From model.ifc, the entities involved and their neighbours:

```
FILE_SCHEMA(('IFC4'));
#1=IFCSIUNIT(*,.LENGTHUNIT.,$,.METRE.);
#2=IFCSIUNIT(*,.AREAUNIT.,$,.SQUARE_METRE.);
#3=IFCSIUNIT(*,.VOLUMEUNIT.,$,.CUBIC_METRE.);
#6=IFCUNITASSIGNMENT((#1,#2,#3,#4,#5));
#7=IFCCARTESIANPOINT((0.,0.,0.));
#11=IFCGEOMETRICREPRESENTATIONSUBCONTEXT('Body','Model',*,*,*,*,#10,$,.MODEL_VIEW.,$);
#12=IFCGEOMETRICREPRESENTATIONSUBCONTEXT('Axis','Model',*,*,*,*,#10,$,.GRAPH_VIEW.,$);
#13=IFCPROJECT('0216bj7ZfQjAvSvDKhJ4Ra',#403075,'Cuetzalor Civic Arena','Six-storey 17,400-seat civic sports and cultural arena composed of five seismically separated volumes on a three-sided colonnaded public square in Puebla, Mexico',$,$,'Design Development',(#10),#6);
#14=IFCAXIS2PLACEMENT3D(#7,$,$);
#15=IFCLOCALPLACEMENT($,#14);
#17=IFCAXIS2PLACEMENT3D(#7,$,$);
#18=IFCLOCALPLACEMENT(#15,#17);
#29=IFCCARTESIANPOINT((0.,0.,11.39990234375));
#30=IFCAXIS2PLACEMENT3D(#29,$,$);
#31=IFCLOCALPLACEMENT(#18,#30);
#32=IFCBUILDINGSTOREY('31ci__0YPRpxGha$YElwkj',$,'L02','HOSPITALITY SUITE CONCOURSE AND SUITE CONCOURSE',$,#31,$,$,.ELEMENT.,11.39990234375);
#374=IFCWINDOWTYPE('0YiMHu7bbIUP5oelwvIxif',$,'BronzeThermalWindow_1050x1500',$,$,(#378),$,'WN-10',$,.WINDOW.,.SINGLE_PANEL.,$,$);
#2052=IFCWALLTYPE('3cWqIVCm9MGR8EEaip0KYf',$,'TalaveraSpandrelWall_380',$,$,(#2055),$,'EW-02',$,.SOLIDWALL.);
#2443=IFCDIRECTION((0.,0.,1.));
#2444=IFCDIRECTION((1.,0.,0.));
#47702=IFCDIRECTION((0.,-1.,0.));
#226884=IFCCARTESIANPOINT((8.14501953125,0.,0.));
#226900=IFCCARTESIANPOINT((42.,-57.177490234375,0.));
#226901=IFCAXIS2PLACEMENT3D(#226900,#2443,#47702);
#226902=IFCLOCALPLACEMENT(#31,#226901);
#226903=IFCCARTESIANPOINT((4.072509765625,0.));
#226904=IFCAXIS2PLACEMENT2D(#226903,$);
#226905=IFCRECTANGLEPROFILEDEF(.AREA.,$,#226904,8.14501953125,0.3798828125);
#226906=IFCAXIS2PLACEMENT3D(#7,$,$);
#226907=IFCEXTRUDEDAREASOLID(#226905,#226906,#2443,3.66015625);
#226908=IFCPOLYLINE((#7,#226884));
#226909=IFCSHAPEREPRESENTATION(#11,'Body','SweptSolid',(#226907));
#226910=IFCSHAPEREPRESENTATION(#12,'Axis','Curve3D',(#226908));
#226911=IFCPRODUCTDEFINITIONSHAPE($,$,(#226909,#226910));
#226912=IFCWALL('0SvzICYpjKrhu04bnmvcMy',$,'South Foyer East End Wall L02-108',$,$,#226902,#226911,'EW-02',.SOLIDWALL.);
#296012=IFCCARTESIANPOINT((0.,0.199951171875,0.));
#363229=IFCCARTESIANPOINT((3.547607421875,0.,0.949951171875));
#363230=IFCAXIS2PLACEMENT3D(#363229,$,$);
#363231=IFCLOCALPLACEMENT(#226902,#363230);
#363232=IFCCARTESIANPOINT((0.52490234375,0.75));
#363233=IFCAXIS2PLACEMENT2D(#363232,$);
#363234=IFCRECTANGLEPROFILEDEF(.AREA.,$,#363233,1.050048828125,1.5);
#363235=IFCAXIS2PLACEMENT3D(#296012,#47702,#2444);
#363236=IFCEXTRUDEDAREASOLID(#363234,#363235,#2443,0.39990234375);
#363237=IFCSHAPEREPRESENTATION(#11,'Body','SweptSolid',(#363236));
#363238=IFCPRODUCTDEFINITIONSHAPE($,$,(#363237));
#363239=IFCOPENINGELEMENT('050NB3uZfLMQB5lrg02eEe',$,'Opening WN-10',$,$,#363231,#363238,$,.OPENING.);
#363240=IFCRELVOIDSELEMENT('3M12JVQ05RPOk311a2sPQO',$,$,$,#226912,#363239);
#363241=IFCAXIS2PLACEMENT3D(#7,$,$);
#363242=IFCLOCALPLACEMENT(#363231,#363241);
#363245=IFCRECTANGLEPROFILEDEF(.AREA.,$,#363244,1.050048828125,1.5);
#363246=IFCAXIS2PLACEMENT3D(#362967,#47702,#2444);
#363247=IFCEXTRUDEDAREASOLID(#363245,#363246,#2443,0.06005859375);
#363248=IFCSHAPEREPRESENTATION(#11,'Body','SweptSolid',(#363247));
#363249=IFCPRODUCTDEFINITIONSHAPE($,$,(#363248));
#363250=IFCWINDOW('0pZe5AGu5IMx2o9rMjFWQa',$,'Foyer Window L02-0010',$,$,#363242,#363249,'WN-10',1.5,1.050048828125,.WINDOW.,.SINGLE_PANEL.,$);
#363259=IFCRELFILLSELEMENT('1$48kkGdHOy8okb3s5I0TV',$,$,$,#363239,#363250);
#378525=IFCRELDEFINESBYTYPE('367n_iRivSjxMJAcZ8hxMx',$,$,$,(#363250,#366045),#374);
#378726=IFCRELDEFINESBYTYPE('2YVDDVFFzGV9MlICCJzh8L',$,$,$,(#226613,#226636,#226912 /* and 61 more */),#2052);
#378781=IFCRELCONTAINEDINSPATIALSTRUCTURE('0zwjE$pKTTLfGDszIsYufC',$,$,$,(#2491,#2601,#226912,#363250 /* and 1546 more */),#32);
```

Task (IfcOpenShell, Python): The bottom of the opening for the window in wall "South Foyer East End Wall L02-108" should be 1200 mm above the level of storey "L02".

```python
import numpy as np
import ifcopenshell
import ifcopenshell.api.geometry
import ifcopenshell.geom
import ifcopenshell.util.element
import ifcopenshell.util.placement
import ifcopenshell.util.shape
import ifcopenshell.util.unit

model = ifcopenshell.open("model.ifc")
unit_scale = ifcopenshell.util.unit.calculate_unit_scale(model)

window = model.by_id(363250)
opening = window.FillsVoids[0].RelatingOpeningElement
storey = ifcopenshell.util.element.get_container(window, ifc_class="IfcBuildingStorey")
level = ifcopenshell.util.placement.get_local_placement(storey.ObjectPlacement)[2, 3]

# The opening's origin need not be at the sill, so measure its lowest point.
shape = ifcopenshell.geom.create_shape(ifcopenshell.geom.settings(), opening)
bottom = ifcopenshell.util.shape.get_shape_bottom_elevation(shape, shape.geometry) / unit_scale
dz = level + 1.2 / unit_scale - bottom

shift = np.array([0.0, 0.0, dz])
# The window is placed relative to its opening, so it follows when the opening moves.
matrix = ifcopenshell.util.placement.get_local_placement(opening.ObjectPlacement)
matrix[:3, 3] += shift
ifcopenshell.api.geometry.edit_object_placement(
    model, product=opening, matrix=matrix, is_si=False, should_transform_children=True
)

print(f"moved by {dz * unit_scale:+.3f} m")

model.write("model_edited.ifc")
```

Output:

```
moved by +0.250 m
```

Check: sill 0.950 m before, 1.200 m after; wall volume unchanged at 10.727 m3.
